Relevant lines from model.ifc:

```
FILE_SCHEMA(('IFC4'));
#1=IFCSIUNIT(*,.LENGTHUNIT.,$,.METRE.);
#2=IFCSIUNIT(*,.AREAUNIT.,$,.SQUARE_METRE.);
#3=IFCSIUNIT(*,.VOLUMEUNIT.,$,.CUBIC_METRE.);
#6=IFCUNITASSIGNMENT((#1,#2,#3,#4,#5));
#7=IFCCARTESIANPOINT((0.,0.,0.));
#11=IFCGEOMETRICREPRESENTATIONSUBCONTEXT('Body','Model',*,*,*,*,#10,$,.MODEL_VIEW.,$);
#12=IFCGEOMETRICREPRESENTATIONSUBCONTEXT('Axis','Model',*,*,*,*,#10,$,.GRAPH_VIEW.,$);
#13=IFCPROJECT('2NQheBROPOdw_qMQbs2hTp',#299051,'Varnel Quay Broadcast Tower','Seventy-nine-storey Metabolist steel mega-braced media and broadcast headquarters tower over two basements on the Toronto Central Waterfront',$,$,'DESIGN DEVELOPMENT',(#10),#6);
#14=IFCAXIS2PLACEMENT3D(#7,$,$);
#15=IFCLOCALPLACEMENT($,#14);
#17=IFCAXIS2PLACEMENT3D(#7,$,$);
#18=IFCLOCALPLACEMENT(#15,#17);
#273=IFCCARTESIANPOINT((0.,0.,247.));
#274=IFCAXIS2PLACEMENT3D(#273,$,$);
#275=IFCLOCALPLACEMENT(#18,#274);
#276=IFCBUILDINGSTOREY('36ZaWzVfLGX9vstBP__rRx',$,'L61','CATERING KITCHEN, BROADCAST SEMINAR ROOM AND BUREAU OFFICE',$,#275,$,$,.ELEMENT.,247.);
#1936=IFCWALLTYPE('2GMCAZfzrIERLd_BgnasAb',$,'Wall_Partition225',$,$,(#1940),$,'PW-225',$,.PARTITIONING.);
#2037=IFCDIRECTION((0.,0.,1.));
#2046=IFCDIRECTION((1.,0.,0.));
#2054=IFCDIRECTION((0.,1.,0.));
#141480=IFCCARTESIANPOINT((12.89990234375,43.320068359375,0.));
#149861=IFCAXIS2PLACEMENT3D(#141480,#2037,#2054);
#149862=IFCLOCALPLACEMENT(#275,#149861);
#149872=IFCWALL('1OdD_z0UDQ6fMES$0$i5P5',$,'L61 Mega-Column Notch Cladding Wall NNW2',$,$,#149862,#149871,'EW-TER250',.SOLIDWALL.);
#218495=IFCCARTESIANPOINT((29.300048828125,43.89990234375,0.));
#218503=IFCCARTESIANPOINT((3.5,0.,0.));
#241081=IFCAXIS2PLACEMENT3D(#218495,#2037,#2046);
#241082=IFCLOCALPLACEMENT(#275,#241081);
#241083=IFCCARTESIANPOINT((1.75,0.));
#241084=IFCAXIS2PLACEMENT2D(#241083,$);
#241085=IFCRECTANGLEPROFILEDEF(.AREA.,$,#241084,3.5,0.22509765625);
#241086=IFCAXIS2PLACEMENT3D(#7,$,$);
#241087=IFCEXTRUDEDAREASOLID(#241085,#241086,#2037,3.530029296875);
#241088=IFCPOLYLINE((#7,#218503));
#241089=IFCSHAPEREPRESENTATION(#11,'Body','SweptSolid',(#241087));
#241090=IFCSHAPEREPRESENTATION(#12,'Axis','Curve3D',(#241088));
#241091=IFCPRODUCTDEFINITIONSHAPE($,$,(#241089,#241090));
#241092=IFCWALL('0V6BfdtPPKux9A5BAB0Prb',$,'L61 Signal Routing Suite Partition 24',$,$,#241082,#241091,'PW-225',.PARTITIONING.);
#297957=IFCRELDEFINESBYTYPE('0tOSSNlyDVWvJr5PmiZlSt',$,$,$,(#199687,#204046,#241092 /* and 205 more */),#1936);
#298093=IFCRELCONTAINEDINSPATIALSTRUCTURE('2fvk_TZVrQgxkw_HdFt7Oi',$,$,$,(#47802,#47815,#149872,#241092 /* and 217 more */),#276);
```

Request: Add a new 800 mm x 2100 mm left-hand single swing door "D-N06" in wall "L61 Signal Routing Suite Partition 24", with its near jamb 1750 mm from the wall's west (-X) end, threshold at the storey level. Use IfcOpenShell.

```python
import numpy as np
import ifcopenshell
import ifcopenshell.api.feature
import ifcopenshell.api.geometry
import ifcopenshell.api.root
import ifcopenshell.api.spatial
import ifcopenshell.geom
import ifcopenshell.util.element
import ifcopenshell.util.placement
import ifcopenshell.util.representation
import ifcopenshell.util.shape
import ifcopenshell.util.unit

model = ifcopenshell.open("model.ifc")
unit_scale = ifcopenshell.util.unit.calculate_unit_scale(model)
settings = ifcopenshell.geom.settings()


def volume(element):
    """Net volume in cubic metres, openings subtracted."""
    shape = ifcopenshell.geom.create_shape(settings, element)
    return ifcopenshell.util.shape.get_volume(shape.geometry)


wall = model.by_id(241092)
storey = ifcopenshell.util.element.get_container(wall, ifc_class="IfcBuildingStorey")
context = ifcopenshell.util.representation.get_context(model, "Model", "Body", "MODEL_VIEW")
before = volume(wall)

width, height, from_end, sill = 0.8, 2.1, 1.75, 0.0  # metres

# The wall runs along its own X axis, and the end named is its -X end.
wall_shape = ifcopenshell.geom.create_shape(settings, wall)
x, y, z = ifcopenshell.util.shape.get_vertices(wall_shape.geometry).T
start = x.min() + from_end
face, thickness = float(y.min()), float(y.max() - y.min())
wall_matrix = ifcopenshell.util.placement.get_local_placement(wall.ObjectPlacement)
level = ifcopenshell.util.placement.get_local_placement(storey.ObjectPlacement)[2, 3]


def in_wall(x, y):
    """Placement at x, y metres in the wall's axes, at sill height."""
    matrix = wall_matrix.copy()
    matrix[:, 3] = wall_matrix @ np.array([x / unit_scale, y / unit_scale, 0.0, 1.0])
    matrix[2, 3] = level + sill / unit_scale
    return matrix


# Opening: a box that overshoots both wall faces by 50 mm.
opening = ifcopenshell.api.root.create_entity(model, ifc_class="IfcOpeningElement", predefined_type="OPENING")
box = ifcopenshell.api.geometry.add_wall_representation(
    model, context=context, length=width, height=height, thickness=thickness + 0.1
)
ifcopenshell.api.geometry.assign_representation(model, product=opening, representation=box)
ifcopenshell.api.geometry.edit_object_placement(model, product=opening, matrix=in_wall(start, face - 0.05), is_si=False)
ifcopenshell.api.feature.add_feature(model, feature=opening, element=wall)

door = ifcopenshell.api.root.create_entity(model, ifc_class="IfcDoor", name="D-N06", predefined_type="DOOR")
door.OverallWidth, door.OverallHeight = width / unit_scale, height / unit_scale
door.OperationType = "SINGLE_SWING_LEFT"
body = ifcopenshell.api.geometry.add_door_representation(
    model,
    context=context,
    overall_width=door.OverallWidth,
    overall_height=door.OverallHeight,
    operation_type="SINGLE_SWING_LEFT",
    lining_properties={"LiningDepth": thickness / unit_scale, "ThresholdDepth": thickness / unit_scale},
)
ifcopenshell.api.geometry.assign_representation(model, product=door, representation=body)
ifcopenshell.api.spatial.assign_container(model, products=[door], relating_structure=storey)
ifcopenshell.api.feature.add_filling(model, opening=opening, element=door)

# The lining spans the wall, so the door starts at the wall face.
ifcopenshell.api.geometry.edit_object_placement(model, product=door, matrix=in_wall(start, face), is_si=False)

after = volume(wall)

print(f"wall volume {before:.3f} -> {after:.3f} m3")

model.write("model_updated.ifc")
```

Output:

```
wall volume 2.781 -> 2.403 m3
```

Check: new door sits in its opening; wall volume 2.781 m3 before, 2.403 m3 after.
